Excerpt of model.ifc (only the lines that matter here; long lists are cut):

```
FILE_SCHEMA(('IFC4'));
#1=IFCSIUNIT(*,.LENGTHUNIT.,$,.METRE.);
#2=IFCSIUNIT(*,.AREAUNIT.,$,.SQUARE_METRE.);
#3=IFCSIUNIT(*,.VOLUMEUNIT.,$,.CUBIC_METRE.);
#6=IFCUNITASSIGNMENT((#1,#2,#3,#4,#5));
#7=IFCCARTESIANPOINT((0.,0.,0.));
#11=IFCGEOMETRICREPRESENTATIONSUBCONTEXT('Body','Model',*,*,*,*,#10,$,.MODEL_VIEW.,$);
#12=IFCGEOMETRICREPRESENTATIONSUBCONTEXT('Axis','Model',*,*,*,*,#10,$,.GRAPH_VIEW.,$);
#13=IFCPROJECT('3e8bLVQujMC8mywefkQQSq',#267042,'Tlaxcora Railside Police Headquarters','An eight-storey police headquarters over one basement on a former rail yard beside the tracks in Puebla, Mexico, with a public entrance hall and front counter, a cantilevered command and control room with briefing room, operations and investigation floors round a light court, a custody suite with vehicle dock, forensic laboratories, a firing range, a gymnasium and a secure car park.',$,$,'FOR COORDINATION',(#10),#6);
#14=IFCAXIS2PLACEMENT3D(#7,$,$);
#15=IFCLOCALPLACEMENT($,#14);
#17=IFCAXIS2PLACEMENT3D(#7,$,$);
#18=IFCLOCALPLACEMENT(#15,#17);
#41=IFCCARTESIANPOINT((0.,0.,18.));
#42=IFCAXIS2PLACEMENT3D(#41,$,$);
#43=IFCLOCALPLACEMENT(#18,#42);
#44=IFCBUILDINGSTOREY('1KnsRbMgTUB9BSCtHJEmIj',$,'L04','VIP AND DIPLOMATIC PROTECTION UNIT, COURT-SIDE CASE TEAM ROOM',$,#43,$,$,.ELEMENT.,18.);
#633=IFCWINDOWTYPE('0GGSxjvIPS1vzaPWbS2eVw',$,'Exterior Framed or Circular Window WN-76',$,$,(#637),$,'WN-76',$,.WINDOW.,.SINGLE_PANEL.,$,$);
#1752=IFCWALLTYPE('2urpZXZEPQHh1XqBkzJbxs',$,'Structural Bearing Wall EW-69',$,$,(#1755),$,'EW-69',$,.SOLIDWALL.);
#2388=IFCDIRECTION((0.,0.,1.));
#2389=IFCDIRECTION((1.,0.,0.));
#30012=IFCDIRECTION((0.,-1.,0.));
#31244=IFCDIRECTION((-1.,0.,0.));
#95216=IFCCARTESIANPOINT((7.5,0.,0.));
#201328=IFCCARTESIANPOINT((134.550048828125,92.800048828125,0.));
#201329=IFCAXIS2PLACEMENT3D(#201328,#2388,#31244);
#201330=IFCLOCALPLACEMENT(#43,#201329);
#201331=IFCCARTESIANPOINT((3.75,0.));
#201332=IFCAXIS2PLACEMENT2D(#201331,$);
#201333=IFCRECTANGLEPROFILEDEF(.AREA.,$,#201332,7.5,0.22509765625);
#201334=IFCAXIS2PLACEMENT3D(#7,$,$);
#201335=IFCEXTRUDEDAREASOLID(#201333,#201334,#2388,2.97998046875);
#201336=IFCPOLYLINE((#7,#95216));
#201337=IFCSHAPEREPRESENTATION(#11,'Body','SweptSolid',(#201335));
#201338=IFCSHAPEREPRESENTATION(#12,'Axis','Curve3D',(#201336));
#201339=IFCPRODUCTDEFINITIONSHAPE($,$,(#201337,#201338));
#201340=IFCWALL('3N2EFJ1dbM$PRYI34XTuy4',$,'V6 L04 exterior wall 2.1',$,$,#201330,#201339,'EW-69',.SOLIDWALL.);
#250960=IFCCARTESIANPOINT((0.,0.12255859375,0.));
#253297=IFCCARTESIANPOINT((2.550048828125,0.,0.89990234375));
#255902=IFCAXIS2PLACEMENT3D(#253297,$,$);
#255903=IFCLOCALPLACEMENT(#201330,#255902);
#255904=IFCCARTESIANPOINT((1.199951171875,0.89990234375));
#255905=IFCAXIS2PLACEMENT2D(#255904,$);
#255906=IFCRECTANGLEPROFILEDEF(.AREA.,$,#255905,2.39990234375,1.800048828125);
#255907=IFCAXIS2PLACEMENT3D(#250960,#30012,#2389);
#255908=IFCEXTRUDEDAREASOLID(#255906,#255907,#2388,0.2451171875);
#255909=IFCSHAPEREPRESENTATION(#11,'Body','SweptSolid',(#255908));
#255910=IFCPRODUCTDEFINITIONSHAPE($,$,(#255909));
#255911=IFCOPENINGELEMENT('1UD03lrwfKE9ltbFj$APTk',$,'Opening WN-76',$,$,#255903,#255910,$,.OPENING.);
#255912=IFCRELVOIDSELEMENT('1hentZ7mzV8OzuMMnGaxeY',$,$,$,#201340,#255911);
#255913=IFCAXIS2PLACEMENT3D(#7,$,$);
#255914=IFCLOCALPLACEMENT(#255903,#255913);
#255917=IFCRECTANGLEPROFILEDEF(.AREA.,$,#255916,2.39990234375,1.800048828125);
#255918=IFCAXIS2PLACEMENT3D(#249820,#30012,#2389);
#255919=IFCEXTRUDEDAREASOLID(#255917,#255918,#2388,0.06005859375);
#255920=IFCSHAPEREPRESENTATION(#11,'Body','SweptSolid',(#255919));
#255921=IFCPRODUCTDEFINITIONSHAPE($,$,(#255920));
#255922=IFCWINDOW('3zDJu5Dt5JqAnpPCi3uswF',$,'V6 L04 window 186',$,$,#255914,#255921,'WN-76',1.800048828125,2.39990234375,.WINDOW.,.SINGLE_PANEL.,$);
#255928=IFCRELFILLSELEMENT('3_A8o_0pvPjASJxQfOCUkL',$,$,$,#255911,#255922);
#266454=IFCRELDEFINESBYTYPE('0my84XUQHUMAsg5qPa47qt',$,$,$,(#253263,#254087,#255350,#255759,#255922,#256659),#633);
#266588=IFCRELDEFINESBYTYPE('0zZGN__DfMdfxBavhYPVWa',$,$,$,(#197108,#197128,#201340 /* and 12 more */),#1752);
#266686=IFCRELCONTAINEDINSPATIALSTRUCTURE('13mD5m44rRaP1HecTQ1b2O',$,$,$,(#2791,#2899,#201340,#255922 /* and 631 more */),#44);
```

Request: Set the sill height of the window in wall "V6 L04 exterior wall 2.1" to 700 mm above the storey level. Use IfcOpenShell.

```python
import numpy as np
import ifcopenshell
import ifcopenshell.api.geometry
import ifcopenshell.geom
import ifcopenshell.util.element
import ifcopenshell.util.placement
import ifcopenshell.util.shape
import ifcopenshell.util.unit

model = ifcopenshell.open("model.ifc")
unit_scale = ifcopenshell.util.unit.calculate_unit_scale(model)

window = model.by_id(255922)
opening = window.FillsVoids[0].RelatingOpeningElement
storey = ifcopenshell.util.element.get_container(window, ifc_class="IfcBuildingStorey")
level = ifcopenshell.util.placement.get_local_placement(storey.ObjectPlacement)[2, 3]

# The opening's origin need not be at the sill, so measure its lowest point.
shape = ifcopenshell.geom.create_shape(ifcopenshell.geom.settings(), opening)
bottom = ifcopenshell.util.shape.get_shape_bottom_elevation(shape, shape.geometry) / unit_scale
dz = level + 0.7 - bottom

shift = np.array([0.0, 0.0, dz])
# The window is placed relative to its opening, so it follows when the opening moves.
matrix = ifcopenshell.util.placement.get_local_placement(opening.ObjectPlacement)
matrix[:3, 3] += shift
ifcopenshell.api.geometry.edit_object_placement(
    model, product=opening, matrix=matrix, is_si=False, should_transform_children=True
)

print(f"moved by {dz * unit_scale:+.3f} m")

model.write("model_rev.ifc")
```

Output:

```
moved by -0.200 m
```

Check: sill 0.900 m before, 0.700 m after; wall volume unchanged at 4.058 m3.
